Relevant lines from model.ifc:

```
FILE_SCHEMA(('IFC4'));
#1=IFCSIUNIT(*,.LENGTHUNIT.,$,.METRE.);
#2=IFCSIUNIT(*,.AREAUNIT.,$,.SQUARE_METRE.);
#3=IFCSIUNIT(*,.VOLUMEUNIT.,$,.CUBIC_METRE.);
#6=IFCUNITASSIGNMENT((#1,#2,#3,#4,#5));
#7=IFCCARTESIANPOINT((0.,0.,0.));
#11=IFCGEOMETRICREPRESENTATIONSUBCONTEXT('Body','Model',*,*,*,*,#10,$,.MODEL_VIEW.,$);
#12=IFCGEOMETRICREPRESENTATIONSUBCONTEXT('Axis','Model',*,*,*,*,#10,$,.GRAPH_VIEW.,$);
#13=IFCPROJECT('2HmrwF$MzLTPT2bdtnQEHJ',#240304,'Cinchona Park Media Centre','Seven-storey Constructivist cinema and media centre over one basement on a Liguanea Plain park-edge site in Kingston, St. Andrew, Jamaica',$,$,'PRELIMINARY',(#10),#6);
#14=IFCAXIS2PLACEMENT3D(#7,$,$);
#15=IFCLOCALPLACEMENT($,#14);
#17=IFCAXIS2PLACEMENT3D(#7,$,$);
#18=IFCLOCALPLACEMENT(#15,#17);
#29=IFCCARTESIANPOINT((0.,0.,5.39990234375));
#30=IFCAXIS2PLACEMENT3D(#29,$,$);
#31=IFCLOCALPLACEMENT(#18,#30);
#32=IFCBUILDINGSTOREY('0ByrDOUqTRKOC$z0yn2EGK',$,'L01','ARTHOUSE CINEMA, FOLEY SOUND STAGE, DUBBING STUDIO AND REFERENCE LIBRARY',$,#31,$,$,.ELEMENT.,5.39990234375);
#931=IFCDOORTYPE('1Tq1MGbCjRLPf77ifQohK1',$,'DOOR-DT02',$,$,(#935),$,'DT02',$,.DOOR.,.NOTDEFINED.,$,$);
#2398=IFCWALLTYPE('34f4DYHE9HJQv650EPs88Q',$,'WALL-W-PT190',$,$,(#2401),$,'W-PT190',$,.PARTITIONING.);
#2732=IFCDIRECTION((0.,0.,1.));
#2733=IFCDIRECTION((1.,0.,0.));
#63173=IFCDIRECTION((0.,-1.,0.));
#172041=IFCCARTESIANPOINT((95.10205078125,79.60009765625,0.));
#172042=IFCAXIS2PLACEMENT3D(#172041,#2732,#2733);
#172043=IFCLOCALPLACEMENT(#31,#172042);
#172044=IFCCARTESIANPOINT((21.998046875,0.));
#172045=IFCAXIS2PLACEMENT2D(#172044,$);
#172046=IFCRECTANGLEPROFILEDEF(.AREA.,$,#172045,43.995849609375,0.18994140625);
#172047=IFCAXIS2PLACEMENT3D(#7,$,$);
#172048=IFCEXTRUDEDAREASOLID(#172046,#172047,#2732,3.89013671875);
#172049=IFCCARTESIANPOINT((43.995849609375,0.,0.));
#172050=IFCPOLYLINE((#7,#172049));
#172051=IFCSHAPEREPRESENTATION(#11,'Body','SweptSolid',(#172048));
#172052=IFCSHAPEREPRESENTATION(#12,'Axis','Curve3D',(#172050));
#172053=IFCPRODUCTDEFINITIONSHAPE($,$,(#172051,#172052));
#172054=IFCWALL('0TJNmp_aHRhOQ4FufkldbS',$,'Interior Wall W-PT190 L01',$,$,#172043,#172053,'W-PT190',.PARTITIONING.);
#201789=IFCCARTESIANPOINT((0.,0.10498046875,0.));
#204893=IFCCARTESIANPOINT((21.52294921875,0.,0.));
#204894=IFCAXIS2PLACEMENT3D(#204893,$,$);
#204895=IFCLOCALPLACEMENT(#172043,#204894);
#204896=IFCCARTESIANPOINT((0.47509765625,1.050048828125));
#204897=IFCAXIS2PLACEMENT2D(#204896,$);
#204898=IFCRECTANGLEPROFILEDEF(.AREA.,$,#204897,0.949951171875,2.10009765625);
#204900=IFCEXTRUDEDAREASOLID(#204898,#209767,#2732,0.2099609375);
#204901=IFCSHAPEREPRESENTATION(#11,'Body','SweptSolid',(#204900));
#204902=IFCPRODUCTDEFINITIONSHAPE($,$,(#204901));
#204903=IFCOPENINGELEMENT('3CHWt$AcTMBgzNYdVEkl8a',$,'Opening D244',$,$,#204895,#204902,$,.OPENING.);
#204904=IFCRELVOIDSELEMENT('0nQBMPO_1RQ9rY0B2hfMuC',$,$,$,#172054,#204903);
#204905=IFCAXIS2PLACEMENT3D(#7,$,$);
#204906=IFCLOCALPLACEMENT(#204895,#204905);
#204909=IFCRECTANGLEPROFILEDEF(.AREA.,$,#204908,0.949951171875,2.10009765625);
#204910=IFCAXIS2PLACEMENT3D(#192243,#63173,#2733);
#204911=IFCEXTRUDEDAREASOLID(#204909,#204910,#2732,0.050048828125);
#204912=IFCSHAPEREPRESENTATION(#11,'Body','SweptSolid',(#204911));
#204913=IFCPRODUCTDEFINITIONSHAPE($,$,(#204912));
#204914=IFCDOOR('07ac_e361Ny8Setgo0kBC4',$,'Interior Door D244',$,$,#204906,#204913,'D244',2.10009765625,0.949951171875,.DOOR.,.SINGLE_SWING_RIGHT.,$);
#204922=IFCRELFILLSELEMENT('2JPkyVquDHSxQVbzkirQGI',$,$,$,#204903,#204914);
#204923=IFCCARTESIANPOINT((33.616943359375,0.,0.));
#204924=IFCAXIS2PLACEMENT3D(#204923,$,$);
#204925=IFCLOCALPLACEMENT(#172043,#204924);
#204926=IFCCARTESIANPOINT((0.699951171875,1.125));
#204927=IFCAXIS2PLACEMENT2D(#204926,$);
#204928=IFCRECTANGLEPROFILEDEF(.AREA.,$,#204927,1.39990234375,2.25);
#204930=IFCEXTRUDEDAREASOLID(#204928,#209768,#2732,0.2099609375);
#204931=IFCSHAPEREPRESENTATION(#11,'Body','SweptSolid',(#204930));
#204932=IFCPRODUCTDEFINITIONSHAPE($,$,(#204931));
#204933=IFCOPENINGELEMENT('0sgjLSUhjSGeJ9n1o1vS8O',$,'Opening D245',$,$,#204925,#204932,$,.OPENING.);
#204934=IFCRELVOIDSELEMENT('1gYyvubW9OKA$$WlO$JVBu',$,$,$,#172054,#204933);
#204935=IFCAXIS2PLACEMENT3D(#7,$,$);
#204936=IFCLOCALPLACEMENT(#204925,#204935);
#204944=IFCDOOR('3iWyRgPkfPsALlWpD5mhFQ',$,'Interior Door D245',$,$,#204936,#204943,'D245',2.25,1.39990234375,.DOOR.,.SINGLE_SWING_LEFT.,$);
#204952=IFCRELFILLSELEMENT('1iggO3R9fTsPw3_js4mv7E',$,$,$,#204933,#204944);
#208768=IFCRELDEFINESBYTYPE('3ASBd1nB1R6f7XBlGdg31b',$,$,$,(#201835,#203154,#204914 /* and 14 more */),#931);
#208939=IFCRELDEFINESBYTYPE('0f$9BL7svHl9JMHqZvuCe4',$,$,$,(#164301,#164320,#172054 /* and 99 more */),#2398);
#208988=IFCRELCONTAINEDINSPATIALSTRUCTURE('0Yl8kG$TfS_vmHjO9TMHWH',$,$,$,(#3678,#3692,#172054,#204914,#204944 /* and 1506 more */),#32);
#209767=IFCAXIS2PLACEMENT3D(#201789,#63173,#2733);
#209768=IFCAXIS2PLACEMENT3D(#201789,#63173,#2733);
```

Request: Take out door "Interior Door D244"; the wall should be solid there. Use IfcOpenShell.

```python
import ifcopenshell
import ifcopenshell.api.feature
import ifcopenshell.api.root
import ifcopenshell.geom
import ifcopenshell.util.shape

model = ifcopenshell.open("model.ifc")
settings = ifcopenshell.geom.settings()


def volume(element):
    """Net volume in cubic metres, openings subtracted."""
    shape = ifcopenshell.geom.create_shape(settings, element)
    return ifcopenshell.util.shape.get_volume(shape.geometry)


door = model.by_guid("07ac_e361Ny8Setgo0kBC4")
opening = door.FillsVoids[0].RelatingOpeningElement
wall = opening.VoidsElements[0].RelatingBuildingElement
before = volume(wall)

ifcopenshell.api.root.remove_product(model, product=door)
ifcopenshell.api.feature.remove_feature(model, feature=opening)

after = volume(wall)

print(f"wall volume {before:.3f} -> {after:.3f} m3")

model.write("model_v2.ifc")
```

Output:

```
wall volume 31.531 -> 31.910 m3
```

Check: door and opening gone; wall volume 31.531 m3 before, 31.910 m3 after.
